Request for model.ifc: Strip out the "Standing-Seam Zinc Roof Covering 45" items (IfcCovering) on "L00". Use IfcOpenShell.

First a look at what the model holds.

```python
import ifcopenshell
import ifcopenshell.util.element

model = ifcopenshell.open("model.ifc")
print(model.schema)
storey = next(s for s in model.by_type("IfcBuildingStorey") if s.Name == "L00")
coverings = [e for e in ifcopenshell.util.element.get_decomposition(storey) if e.is_a("IfcCovering")]
seen = {}
for e in coverings:
    element_type = ifcopenshell.util.element.get_type(e)
    name = element_type.Name if element_type not in (None, e) else None
    seen[name] = seen.get(name, 0) + 1
for name, count in sorted(seen.items(), key=str):
    print(count, "x", name)
```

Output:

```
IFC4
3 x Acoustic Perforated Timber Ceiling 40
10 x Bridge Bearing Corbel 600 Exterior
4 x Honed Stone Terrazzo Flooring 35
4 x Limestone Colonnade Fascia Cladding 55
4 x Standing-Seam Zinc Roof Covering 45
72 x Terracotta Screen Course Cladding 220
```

```python
import ifcopenshell
import ifcopenshell.api.root
import ifcopenshell.util.element

model = ifcopenshell.open("model.ifc")

storey = next(s for s in model.by_type("IfcBuildingStorey") if s.Name == "L00")
coverings = [e for e in ifcopenshell.util.element.get_decomposition(storey) if e.is_a("IfcCovering")]
targets = [e for e in coverings if (t := ifcopenshell.util.element.get_type(e)) not in (None, e) and t.Name == "Standing-Seam Zinc Roof Covering 45"]

for e in targets:
    ifcopenshell.api.root.remove_product(model, product=e)
print(len(targets), "removed")

model.write("model_updated.ifc")
```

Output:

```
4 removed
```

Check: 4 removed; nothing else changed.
